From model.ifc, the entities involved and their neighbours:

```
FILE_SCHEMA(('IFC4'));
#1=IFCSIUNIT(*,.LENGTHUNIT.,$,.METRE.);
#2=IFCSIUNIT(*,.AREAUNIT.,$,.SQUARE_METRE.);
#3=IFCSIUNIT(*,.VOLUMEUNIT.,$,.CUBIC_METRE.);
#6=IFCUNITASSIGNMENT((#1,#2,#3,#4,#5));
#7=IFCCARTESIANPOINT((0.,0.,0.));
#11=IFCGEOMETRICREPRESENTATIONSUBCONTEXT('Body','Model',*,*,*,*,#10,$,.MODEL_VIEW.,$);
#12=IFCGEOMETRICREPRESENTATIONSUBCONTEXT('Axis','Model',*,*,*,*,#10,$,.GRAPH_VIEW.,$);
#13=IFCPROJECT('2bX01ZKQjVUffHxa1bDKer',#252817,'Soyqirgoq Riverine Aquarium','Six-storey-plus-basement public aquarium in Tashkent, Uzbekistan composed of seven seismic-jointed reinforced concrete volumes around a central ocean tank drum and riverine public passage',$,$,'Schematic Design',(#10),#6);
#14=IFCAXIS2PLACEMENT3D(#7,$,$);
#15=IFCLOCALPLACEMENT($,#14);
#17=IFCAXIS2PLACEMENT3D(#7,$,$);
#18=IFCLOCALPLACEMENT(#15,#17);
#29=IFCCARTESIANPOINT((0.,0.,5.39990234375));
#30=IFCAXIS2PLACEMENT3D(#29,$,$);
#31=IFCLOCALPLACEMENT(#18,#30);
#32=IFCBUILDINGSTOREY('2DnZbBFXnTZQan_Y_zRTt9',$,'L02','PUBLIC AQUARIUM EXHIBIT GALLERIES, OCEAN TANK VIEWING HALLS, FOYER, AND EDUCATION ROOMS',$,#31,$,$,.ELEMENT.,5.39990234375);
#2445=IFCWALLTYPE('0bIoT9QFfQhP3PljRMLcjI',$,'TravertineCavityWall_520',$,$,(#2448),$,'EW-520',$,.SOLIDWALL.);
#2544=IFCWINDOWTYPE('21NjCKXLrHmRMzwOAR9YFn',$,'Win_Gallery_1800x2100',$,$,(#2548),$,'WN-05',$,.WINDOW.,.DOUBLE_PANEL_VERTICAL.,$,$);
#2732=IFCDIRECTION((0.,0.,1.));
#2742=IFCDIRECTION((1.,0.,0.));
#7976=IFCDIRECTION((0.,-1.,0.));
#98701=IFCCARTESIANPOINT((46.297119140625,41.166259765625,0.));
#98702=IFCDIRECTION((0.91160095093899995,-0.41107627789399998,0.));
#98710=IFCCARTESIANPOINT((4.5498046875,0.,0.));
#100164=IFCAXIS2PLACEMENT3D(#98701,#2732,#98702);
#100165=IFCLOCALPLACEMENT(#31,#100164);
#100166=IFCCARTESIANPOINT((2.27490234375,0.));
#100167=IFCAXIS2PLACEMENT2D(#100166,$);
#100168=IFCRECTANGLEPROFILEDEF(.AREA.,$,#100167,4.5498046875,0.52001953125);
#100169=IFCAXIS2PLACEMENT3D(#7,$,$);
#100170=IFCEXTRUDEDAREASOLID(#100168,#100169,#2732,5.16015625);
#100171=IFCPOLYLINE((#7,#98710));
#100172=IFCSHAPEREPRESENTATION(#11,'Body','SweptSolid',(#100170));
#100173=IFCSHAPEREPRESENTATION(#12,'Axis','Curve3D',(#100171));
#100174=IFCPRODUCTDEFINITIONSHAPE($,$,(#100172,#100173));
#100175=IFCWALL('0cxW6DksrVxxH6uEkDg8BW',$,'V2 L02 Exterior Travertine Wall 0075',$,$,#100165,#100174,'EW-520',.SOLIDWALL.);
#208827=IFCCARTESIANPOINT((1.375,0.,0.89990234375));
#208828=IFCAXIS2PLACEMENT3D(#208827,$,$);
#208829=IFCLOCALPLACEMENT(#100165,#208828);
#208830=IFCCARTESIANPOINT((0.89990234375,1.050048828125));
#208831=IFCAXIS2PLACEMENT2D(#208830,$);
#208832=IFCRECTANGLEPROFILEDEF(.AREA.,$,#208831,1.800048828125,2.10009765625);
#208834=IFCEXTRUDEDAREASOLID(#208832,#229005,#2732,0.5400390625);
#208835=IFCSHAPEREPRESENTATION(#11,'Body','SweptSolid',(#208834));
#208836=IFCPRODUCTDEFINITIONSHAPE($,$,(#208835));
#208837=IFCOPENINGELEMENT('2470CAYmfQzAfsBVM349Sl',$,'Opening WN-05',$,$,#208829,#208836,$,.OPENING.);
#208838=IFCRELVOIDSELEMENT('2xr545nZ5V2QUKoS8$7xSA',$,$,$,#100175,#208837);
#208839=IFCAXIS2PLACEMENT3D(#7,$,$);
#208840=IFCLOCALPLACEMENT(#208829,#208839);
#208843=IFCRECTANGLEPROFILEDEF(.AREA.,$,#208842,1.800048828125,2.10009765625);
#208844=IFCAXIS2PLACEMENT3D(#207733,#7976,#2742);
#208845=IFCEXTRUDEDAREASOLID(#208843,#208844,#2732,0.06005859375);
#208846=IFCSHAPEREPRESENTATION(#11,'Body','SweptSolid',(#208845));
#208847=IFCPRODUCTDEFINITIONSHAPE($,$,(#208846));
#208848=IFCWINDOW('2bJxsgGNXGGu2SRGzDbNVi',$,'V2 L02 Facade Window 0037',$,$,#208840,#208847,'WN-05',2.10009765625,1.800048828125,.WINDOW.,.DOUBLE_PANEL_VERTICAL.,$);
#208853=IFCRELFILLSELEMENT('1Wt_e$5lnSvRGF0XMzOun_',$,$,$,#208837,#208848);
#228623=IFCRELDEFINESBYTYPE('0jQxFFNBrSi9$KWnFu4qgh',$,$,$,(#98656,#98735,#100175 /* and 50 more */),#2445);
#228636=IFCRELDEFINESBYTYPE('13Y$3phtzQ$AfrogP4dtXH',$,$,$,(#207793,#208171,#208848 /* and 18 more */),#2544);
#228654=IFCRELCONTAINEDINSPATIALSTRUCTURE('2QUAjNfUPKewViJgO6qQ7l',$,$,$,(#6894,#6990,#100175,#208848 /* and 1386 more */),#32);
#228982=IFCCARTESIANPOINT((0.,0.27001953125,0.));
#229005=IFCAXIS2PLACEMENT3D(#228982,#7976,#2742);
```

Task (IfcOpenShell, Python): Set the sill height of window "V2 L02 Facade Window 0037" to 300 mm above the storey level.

```python
import numpy as np
import ifcopenshell
import ifcopenshell.api.geometry
import ifcopenshell.geom
import ifcopenshell.util.element
import ifcopenshell.util.placement
import ifcopenshell.util.shape
import ifcopenshell.util.unit

model = ifcopenshell.open("model.ifc")
unit_scale = ifcopenshell.util.unit.calculate_unit_scale(model)

window = model.by_guid("2bJxsgGNXGGu2SRGzDbNVi")
opening = window.FillsVoids[0].RelatingOpeningElement
storey = ifcopenshell.util.element.get_container(window, ifc_class="IfcBuildingStorey")
level = ifcopenshell.util.placement.get_local_placement(storey.ObjectPlacement)[2, 3]

# The opening's origin need not be at the sill, so measure its lowest point.
shape = ifcopenshell.geom.create_shape(ifcopenshell.geom.settings(), opening)
bottom = ifcopenshell.util.shape.get_shape_bottom_elevation(shape, shape.geometry) / unit_scale
dz = level + 0.3 / unit_scale - bottom

shift = np.array([0.0, 0.0, dz])
# The window is placed relative to its opening, so it follows when the opening moves.
matrix = ifcopenshell.util.placement.get_local_placement(opening.ObjectPlacement)
matrix[:3, 3] += shift
ifcopenshell.api.geometry.edit_object_placement(
    model, product=opening, matrix=matrix, is_si=False, should_transform_children=True
)

print(f"moved by {dz * unit_scale:+.3f} m")

model.write("model_updated.ifc")
```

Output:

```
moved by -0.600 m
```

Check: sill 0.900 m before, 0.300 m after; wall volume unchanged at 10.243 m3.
